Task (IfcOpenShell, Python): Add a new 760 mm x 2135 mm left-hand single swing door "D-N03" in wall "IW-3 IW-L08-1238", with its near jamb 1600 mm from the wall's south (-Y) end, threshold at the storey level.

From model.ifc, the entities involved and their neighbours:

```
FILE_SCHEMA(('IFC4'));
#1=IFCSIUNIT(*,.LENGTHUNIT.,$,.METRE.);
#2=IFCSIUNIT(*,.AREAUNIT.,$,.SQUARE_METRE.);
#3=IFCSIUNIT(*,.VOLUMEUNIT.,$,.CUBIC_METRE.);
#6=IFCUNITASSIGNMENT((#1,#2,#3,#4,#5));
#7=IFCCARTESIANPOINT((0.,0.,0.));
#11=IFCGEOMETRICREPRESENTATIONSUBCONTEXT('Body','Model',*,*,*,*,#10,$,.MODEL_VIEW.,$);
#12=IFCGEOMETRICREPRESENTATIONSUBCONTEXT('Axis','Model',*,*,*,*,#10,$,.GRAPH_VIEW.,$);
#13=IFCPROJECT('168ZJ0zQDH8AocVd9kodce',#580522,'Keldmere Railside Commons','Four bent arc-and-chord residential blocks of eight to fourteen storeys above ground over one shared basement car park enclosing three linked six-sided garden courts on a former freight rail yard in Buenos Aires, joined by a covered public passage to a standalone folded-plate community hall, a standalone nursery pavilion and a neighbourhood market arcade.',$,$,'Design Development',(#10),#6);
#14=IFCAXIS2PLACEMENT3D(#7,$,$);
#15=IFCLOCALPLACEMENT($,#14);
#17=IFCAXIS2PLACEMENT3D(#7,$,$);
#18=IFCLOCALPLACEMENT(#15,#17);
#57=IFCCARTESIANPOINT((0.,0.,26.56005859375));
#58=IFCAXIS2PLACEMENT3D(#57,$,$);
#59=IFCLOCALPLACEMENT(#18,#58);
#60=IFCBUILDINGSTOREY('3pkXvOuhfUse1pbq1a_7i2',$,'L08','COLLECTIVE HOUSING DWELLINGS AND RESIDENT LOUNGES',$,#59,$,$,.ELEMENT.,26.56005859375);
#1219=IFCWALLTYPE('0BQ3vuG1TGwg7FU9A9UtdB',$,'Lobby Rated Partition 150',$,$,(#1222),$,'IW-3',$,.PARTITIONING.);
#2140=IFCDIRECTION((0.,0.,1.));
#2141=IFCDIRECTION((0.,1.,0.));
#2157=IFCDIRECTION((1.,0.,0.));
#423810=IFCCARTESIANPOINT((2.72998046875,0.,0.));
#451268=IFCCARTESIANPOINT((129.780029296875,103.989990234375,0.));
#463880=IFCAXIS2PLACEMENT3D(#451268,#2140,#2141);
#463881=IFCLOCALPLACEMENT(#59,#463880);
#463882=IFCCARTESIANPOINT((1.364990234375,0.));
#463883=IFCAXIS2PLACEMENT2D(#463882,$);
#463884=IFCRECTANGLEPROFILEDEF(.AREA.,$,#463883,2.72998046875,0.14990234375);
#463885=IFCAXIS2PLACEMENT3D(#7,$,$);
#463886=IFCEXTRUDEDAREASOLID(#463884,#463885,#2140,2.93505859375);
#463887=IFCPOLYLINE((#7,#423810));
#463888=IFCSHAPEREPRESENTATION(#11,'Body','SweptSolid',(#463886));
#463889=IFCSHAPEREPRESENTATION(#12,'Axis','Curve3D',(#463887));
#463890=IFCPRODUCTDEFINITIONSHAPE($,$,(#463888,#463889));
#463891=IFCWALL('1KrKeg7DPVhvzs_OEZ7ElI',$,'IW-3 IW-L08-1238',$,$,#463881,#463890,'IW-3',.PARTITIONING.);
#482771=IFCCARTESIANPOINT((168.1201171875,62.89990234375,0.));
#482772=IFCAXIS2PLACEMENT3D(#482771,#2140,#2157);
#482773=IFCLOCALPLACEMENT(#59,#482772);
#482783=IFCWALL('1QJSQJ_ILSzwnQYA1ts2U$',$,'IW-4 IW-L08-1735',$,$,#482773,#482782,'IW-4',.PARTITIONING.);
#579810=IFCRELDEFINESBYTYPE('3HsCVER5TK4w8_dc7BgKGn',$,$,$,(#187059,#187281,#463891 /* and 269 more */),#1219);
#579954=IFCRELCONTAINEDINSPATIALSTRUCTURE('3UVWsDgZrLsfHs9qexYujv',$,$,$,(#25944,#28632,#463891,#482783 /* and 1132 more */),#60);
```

```python
import numpy as np
import ifcopenshell
import ifcopenshell.api.feature
import ifcopenshell.api.geometry
import ifcopenshell.api.root
import ifcopenshell.api.spatial
import ifcopenshell.geom
import ifcopenshell.util.element
import ifcopenshell.util.placement
import ifcopenshell.util.representation
import ifcopenshell.util.shape
import ifcopenshell.util.unit

model = ifcopenshell.open("model.ifc")
unit_scale = ifcopenshell.util.unit.calculate_unit_scale(model)
settings = ifcopenshell.geom.settings()


def volume(element):
    """Net volume in cubic metres, openings subtracted."""
    shape = ifcopenshell.geom.create_shape(settings, element)
    return ifcopenshell.util.shape.get_volume(shape.geometry)


wall = model.by_guid("1KrKeg7DPVhvzs_OEZ7ElI")
storey = ifcopenshell.util.element.get_container(wall, ifc_class="IfcBuildingStorey")
context = ifcopenshell.util.representation.get_context(model, "Model", "Body", "MODEL_VIEW")
before = volume(wall)

width, height, from_end, sill = 0.76, 2.135, 1.6, 0.0  # metres

# The wall runs along its own X axis, and the end named is its -X end.
wall_shape = ifcopenshell.geom.create_shape(settings, wall)
x, y, z = ifcopenshell.util.shape.get_vertices(wall_shape.geometry).T
start = x.min() + from_end
face, thickness = float(y.min()), float(y.max() - y.min())
wall_matrix = ifcopenshell.util.placement.get_local_placement(wall.ObjectPlacement)
level = ifcopenshell.util.placement.get_local_placement(storey.ObjectPlacement)[2, 3]


def in_wall(x, y):
    """Placement at x, y metres in the wall's axes, at sill height."""
    matrix = wall_matrix.copy()
    matrix[:, 3] = wall_matrix @ np.array([x / unit_scale, y / unit_scale, 0.0, 1.0])
    matrix[2, 3] = level + sill / unit_scale
    return matrix


# Opening: a box that overshoots both wall faces by 50 mm.
opening = ifcopenshell.api.root.create_entity(model, ifc_class="IfcOpeningElement", predefined_type="OPENING")
box = ifcopenshell.api.geometry.add_wall_representation(
    model, context=context, length=width, height=height, thickness=thickness + 0.1
)
ifcopenshell.api.geometry.assign_representation(model, product=opening, representation=box)
ifcopenshell.api.geometry.edit_object_placement(model, product=opening, matrix=in_wall(start, face - 0.05), is_si=False)
ifcopenshell.api.feature.add_feature(model, feature=opening, element=wall)

door = ifcopenshell.api.root.create_entity(model, ifc_class="IfcDoor", name="D-N03", predefined_type="DOOR")
door.OverallWidth, door.OverallHeight = width / unit_scale, height / unit_scale
door.OperationType = "SINGLE_SWING_LEFT"
body = ifcopenshell.api.geometry.add_door_representation(
    model,
    context=context,
    overall_width=door.OverallWidth,
    overall_height=door.OverallHeight,
    operation_type="SINGLE_SWING_LEFT",
    lining_properties={"LiningDepth": thickness / unit_scale, "ThresholdDepth": thickness / unit_scale},
)
ifcopenshell.api.geometry.assign_representation(model, product=door, representation=body)
ifcopenshell.api.spatial.assign_container(model, products=[door], relating_structure=storey)
ifcopenshell.api.feature.add_filling(model, opening=opening, element=door)

# The lining spans the wall, so the door starts at the wall face.
ifcopenshell.api.geometry.edit_object_placement(model, product=door, matrix=in_wall(start, face), is_si=False)

after = volume(wall)

print(f"wall volume {before:.3f} -> {after:.3f} m3")

model.write("model_v2.ifc")
```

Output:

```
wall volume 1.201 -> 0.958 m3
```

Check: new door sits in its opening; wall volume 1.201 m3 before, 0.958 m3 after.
